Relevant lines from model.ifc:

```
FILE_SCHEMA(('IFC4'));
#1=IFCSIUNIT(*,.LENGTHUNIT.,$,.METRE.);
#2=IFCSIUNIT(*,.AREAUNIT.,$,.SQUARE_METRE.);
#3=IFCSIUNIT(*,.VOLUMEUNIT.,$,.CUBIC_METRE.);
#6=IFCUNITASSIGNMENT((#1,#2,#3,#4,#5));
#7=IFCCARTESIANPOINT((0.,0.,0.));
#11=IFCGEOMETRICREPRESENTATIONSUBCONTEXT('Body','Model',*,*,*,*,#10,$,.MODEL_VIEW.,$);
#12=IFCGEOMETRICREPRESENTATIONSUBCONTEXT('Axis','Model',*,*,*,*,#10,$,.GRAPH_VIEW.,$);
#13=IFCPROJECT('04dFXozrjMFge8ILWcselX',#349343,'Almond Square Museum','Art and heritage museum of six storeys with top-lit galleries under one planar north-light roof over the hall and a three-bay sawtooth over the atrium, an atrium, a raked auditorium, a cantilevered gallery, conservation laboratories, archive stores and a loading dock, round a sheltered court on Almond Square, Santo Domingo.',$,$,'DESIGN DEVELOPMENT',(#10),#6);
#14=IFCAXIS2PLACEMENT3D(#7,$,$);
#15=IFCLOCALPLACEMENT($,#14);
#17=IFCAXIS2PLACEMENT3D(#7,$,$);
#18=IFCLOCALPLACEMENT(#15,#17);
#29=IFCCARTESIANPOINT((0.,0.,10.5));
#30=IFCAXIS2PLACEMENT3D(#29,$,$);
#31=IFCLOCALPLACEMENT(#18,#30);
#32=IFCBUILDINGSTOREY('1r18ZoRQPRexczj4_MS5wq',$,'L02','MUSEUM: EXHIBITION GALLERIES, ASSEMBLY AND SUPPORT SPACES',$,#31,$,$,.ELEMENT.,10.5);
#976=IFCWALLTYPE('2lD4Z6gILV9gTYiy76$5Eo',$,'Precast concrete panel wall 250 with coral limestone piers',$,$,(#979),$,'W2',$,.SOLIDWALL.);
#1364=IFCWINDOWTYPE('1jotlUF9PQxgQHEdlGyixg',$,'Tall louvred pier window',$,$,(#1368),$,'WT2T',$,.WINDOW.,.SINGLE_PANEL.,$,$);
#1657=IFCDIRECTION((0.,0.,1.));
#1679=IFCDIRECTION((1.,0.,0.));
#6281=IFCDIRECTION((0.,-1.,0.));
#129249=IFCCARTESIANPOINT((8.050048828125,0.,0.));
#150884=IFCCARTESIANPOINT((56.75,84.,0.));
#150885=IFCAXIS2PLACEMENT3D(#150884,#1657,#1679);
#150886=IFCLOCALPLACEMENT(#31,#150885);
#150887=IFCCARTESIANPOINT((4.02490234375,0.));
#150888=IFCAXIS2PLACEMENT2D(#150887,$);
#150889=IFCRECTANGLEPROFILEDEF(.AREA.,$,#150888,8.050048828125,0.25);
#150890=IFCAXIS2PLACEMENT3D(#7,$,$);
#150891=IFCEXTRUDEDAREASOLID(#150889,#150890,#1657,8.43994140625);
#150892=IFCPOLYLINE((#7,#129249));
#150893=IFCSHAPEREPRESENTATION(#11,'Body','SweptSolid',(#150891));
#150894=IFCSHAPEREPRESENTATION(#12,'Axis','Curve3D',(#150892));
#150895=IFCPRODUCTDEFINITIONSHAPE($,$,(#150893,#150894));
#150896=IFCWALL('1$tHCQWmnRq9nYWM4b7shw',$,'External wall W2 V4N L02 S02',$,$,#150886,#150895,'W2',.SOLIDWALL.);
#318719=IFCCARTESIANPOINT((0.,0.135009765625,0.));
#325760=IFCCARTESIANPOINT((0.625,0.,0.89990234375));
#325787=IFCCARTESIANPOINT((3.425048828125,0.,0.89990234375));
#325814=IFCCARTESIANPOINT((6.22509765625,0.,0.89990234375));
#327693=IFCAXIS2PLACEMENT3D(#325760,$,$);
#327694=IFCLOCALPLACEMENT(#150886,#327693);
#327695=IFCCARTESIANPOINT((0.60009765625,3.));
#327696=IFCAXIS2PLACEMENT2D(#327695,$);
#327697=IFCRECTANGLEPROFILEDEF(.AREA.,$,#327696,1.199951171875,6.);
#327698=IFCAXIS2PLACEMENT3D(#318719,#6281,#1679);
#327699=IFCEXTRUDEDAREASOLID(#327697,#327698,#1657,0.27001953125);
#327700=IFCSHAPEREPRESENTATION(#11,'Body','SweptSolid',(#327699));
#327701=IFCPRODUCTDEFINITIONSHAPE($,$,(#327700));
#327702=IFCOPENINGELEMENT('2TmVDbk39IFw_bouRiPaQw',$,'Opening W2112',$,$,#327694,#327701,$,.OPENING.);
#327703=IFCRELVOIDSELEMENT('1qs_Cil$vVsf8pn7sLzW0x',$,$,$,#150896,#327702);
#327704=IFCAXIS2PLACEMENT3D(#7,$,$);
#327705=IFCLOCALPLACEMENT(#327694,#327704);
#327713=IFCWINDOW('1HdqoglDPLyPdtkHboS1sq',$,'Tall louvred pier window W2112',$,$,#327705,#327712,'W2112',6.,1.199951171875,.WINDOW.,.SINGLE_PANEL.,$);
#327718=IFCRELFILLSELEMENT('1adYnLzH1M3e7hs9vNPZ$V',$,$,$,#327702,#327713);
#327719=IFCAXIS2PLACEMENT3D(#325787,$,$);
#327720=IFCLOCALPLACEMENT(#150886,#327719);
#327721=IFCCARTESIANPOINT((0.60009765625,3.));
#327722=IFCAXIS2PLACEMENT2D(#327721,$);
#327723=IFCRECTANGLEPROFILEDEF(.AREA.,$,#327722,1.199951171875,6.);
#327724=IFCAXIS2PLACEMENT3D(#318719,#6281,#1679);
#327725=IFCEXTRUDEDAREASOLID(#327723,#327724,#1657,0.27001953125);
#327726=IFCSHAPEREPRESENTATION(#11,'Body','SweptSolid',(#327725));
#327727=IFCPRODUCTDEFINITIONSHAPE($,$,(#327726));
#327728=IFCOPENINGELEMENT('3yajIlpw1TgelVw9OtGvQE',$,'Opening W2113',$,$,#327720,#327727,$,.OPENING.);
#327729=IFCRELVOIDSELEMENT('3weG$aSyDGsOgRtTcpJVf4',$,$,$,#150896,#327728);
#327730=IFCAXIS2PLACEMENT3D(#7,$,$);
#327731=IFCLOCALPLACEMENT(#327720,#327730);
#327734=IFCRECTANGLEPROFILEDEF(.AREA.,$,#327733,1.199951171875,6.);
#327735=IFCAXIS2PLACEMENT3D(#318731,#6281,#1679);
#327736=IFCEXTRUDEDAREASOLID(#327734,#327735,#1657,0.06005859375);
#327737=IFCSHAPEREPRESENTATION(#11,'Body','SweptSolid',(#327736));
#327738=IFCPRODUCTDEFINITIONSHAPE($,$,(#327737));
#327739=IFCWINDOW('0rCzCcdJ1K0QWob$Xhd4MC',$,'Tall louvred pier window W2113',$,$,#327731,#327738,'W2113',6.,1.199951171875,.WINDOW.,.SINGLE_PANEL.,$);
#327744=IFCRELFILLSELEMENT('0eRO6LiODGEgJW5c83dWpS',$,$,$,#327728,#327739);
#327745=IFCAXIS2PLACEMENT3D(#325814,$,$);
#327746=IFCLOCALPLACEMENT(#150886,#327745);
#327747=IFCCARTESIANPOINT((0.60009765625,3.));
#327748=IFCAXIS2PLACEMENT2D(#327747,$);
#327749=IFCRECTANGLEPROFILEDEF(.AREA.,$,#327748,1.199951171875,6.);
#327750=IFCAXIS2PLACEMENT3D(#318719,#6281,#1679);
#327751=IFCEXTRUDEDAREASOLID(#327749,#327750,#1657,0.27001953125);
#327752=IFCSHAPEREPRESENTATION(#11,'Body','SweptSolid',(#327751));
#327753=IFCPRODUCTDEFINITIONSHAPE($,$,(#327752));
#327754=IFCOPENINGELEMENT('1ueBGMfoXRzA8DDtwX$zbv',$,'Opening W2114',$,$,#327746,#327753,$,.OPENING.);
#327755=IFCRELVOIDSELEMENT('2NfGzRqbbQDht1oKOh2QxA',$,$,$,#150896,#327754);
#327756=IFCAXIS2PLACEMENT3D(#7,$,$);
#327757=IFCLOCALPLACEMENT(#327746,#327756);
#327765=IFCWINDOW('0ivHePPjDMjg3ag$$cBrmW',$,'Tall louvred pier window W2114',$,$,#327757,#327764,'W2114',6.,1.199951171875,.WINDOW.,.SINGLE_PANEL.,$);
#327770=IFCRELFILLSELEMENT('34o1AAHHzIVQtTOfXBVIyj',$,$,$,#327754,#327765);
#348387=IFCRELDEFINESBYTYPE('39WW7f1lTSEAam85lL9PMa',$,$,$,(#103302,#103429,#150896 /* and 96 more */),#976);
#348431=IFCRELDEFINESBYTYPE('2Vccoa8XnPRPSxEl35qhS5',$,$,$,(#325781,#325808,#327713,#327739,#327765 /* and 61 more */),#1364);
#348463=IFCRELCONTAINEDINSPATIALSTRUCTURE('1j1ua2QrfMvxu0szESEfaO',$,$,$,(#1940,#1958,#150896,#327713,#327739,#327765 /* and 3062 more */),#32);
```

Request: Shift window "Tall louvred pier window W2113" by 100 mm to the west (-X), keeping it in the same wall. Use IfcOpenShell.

```python
import ifcopenshell
import ifcopenshell.api.geometry
import ifcopenshell.util.placement
import ifcopenshell.util.unit

model = ifcopenshell.open("model.ifc")
unit_scale = ifcopenshell.util.unit.calculate_unit_scale(model)

window = model.by_guid("0rCzCcdJ1K0QWob$Xhd4MC")
opening = window.FillsVoids[0].RelatingOpeningElement
wall = opening.VoidsElements[0].RelatingBuildingElement

wall_matrix = ifcopenshell.util.placement.get_local_placement(wall.ObjectPlacement)
shift = wall_matrix[:3, 0] * -0.1 / unit_scale
before = ifcopenshell.util.placement.get_local_placement(window.ObjectPlacement)[:3, 3].copy()

# The window is placed relative to its opening, so it follows when the opening moves.
matrix = ifcopenshell.util.placement.get_local_placement(opening.ObjectPlacement)
matrix[:3, 3] += shift
ifcopenshell.api.geometry.edit_object_placement(
    model, product=opening, matrix=matrix, is_si=False, should_transform_children=True
)

after = ifcopenshell.util.placement.get_local_placement(window.ObjectPlacement)[:3, 3]
print("window moved by", (after - before).round(3) + 0.0)

model.write("model-out.ifc")
```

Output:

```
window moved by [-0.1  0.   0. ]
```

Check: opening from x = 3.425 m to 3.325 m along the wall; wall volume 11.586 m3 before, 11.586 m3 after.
